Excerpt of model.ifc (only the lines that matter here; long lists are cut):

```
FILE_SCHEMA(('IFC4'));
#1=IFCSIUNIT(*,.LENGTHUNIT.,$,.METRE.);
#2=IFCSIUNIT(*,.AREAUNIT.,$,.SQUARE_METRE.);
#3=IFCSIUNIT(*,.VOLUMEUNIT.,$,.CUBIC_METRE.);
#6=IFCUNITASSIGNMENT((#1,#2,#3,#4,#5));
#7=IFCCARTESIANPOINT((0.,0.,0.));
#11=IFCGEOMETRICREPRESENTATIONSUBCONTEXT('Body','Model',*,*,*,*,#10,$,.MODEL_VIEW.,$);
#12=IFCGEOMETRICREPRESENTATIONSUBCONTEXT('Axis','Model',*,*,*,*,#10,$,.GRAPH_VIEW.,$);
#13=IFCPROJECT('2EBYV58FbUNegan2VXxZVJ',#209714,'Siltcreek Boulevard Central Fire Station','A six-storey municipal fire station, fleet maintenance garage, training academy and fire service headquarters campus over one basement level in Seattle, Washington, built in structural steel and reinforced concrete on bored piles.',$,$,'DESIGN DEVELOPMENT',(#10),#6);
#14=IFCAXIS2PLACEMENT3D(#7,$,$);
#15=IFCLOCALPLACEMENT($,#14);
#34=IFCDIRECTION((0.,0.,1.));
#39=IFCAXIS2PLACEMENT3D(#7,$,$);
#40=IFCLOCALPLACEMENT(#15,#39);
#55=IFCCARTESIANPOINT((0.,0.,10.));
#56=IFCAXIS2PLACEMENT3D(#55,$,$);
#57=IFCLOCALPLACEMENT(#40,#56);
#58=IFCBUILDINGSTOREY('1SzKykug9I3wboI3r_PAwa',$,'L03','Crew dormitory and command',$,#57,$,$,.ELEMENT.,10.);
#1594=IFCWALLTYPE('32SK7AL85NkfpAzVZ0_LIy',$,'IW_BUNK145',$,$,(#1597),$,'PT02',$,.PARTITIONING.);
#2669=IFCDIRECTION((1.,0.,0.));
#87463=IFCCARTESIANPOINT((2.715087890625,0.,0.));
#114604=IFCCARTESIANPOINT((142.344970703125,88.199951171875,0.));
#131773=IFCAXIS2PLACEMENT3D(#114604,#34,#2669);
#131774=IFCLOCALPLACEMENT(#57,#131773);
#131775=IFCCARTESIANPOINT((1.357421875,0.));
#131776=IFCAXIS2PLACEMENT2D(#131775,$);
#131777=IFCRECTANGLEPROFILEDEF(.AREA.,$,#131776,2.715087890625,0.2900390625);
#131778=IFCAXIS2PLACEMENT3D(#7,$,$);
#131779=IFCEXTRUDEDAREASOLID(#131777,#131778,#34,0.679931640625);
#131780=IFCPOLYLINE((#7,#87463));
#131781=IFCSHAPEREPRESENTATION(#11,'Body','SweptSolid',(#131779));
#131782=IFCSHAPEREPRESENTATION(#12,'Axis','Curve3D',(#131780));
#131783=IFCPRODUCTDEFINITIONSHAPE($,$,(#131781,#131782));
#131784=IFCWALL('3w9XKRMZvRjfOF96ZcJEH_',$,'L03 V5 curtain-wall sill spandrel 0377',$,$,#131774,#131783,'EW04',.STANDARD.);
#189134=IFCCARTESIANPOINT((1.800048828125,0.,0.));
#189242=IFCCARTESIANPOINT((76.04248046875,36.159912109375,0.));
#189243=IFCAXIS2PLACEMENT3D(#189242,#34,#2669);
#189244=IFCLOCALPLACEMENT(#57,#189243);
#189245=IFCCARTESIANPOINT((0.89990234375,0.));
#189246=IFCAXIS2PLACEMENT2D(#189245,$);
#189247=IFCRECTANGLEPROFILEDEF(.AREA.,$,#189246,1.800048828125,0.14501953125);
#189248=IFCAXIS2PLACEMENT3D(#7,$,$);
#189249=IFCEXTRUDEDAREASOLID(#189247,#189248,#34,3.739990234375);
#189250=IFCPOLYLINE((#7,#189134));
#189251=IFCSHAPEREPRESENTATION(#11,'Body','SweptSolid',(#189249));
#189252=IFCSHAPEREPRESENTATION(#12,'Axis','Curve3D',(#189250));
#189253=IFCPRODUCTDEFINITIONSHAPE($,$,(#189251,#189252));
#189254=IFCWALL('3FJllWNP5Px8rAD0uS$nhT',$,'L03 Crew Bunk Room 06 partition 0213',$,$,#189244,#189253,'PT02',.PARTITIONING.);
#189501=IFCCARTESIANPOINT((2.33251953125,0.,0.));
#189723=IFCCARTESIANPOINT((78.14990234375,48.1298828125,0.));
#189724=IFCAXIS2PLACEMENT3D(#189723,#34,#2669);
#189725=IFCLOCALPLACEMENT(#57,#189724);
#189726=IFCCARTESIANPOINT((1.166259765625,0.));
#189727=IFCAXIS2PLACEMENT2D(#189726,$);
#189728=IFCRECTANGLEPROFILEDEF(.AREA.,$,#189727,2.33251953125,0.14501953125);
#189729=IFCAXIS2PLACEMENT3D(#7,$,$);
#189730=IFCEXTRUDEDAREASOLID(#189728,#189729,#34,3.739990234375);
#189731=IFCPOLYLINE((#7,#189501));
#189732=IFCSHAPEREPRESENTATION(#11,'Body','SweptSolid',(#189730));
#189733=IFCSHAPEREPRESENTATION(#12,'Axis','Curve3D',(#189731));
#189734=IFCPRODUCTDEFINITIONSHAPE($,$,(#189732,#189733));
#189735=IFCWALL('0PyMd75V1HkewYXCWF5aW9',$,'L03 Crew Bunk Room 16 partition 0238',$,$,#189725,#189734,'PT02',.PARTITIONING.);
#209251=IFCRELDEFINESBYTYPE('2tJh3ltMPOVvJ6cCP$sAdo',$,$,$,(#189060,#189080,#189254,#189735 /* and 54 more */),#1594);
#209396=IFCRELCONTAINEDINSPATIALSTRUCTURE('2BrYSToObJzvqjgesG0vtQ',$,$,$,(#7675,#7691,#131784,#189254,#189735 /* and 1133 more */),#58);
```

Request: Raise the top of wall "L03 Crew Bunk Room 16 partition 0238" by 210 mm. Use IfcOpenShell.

```python
import ifcopenshell
import ifcopenshell.geom
import ifcopenshell.util.representation
import ifcopenshell.util.shape
import ifcopenshell.util.unit

model = ifcopenshell.open("model.ifc")
unit_scale = ifcopenshell.util.unit.calculate_unit_scale(model)
settings = ifcopenshell.geom.settings()


def volume(element):
    """Net volume in cubic metres, openings subtracted."""
    shape = ifcopenshell.geom.create_shape(settings, element)
    return ifcopenshell.util.shape.get_volume(shape.geometry)


wall = model.by_id(189735)
before = volume(wall)

body = ifcopenshell.util.representation.get_representation(wall, "Model", "Body")
solid = body.Items[0]
old_height = solid.Depth
solid.Depth += 0.21 / unit_scale
after = volume(wall)

print(f"height {old_height:g} -> {solid.Depth:g}, volume {before:.3f} -> {after:.3f} m3")

model.write("model_rev.ifc")
```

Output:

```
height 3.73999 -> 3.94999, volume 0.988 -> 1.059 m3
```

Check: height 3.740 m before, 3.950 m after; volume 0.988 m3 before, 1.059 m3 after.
